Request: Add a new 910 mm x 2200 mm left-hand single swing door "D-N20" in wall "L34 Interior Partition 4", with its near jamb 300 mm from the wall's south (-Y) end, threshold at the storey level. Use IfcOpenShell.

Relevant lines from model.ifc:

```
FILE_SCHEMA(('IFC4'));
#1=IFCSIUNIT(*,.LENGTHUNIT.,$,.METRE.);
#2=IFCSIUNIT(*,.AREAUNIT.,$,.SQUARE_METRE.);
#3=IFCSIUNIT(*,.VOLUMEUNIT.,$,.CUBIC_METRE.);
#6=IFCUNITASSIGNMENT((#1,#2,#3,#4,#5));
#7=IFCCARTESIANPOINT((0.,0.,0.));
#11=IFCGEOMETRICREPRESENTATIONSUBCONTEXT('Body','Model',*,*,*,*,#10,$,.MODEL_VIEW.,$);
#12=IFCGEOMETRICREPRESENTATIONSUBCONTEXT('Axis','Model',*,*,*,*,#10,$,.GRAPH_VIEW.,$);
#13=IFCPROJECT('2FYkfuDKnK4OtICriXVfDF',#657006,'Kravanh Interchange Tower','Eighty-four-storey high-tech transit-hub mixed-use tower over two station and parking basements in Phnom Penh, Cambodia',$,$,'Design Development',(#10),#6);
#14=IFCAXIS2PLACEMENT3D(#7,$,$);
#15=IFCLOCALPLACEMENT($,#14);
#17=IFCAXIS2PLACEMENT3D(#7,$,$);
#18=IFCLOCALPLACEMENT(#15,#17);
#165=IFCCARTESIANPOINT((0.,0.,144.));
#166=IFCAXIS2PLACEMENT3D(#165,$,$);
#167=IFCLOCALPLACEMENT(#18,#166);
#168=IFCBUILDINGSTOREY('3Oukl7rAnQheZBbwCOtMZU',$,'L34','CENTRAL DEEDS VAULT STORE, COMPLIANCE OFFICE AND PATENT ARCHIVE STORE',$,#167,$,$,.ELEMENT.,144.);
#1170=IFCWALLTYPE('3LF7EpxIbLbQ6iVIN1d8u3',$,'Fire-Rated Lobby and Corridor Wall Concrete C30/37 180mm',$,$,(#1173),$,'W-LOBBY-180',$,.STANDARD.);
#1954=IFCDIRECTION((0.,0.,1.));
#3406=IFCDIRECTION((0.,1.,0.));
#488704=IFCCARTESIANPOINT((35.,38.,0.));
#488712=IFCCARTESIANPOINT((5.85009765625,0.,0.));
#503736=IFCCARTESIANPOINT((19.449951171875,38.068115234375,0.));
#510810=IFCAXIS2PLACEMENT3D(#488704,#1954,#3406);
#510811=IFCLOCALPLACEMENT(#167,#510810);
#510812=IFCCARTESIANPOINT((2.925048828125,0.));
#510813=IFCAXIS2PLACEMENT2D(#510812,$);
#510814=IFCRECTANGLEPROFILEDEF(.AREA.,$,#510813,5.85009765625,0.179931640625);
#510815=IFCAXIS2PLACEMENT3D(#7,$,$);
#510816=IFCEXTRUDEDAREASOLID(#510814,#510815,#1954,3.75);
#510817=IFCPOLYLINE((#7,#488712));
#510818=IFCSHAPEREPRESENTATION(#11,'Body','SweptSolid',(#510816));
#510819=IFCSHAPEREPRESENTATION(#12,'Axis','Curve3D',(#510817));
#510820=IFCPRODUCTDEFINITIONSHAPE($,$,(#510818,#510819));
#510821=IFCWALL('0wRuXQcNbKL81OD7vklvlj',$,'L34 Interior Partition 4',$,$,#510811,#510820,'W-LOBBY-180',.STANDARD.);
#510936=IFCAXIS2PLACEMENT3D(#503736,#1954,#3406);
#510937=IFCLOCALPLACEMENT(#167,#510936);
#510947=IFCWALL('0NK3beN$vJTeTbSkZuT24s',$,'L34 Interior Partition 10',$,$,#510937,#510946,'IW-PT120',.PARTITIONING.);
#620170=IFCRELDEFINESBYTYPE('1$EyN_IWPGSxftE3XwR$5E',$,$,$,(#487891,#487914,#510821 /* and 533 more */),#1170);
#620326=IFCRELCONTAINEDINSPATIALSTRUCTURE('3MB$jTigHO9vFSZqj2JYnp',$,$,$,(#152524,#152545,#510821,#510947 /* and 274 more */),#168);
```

```python
import numpy as np
import ifcopenshell
import ifcopenshell.api.feature
import ifcopenshell.api.geometry
import ifcopenshell.api.root
import ifcopenshell.api.spatial
import ifcopenshell.geom
import ifcopenshell.util.element
import ifcopenshell.util.placement
import ifcopenshell.util.representation
import ifcopenshell.util.shape
import ifcopenshell.util.unit

model = ifcopenshell.open("model.ifc")
unit_scale = ifcopenshell.util.unit.calculate_unit_scale(model)
settings = ifcopenshell.geom.settings()


def volume(element):
    """Net volume in cubic metres, openings subtracted."""
    shape = ifcopenshell.geom.create_shape(settings, element)
    return ifcopenshell.util.shape.get_volume(shape.geometry)


wall = model.by_guid("0wRuXQcNbKL81OD7vklvlj")
storey = ifcopenshell.util.element.get_container(wall, ifc_class="IfcBuildingStorey")
context = ifcopenshell.util.representation.get_context(model, "Model", "Body", "MODEL_VIEW")
before = volume(wall)

width, height, from_end, sill = 0.91, 2.2, 0.3, 0.0  # metres

# The wall runs along its own X axis, and the end named is its -X end.
wall_shape = ifcopenshell.geom.create_shape(settings, wall)
x, y, z = ifcopenshell.util.shape.get_vertices(wall_shape.geometry).T
start = x.min() + from_end
face, thickness = float(y.min()), float(y.max() - y.min())
wall_matrix = ifcopenshell.util.placement.get_local_placement(wall.ObjectPlacement)
level = ifcopenshell.util.placement.get_local_placement(storey.ObjectPlacement)[2, 3]


def in_wall(x, y):
    """Placement at x, y metres in the wall's axes, at sill height."""
    matrix = wall_matrix.copy()
    matrix[:, 3] = wall_matrix @ np.array([x / unit_scale, y / unit_scale, 0.0, 1.0])
    matrix[2, 3] = level + sill / unit_scale
    return matrix


# Opening: a box that overshoots both wall faces by 50 mm.
opening = ifcopenshell.api.root.create_entity(model, ifc_class="IfcOpeningElement", predefined_type="OPENING")
box = ifcopenshell.api.geometry.add_wall_representation(
    model, context=context, length=width, height=height, thickness=thickness + 0.1
)
ifcopenshell.api.geometry.assign_representation(model, product=opening, representation=box)
ifcopenshell.api.geometry.edit_object_placement(model, product=opening, matrix=in_wall(start, face - 0.05), is_si=False)
ifcopenshell.api.feature.add_feature(model, feature=opening, element=wall)

door = ifcopenshell.api.root.create_entity(model, ifc_class="IfcDoor", name="D-N20", predefined_type="DOOR")
door.OverallWidth, door.OverallHeight = width / unit_scale, height / unit_scale
door.OperationType = "SINGLE_SWING_LEFT"
body = ifcopenshell.api.geometry.add_door_representation(
    model,
    context=context,
    overall_width=door.OverallWidth,
    overall_height=door.OverallHeight,
    operation_type="SINGLE_SWING_LEFT",
    lining_properties={"LiningDepth": thickness / unit_scale, "ThresholdDepth": thickness / unit_scale},
)
ifcopenshell.api.geometry.assign_representation(model, product=door, representation=body)
ifcopenshell.api.spatial.assign_container(model, products=[door], relating_structure=storey)
ifcopenshell.api.feature.add_filling(model, opening=opening, element=door)

# The lining spans the wall, so the door starts at the wall face.
ifcopenshell.api.geometry.edit_object_placement(model, product=door, matrix=in_wall(start, face), is_si=False)

after = volume(wall)

print(f"wall volume {before:.3f} -> {after:.3f} m3")

model.write("model_edited.ifc")
```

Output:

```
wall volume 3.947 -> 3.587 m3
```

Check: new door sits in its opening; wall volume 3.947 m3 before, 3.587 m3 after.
